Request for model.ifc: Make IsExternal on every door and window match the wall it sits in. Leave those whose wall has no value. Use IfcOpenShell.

First a look at what the model holds.

```python
import ifcopenshell
import ifcopenshell.util.element

model = ifcopenshell.open("model.ifc")
print(model.schema)
seen = {}
for e in model.by_type("IfcDoor") + model.by_type("IfcWindow"):
    if not e.FillsVoids:
        continue
    host = e.FillsVoids[0].RelatingOpeningElement.VoidsElements[0].RelatingBuildingElement
    own = ifcopenshell.util.element.get_pset(e, f"Pset_{e.is_a()[3:].removesuffix('StandardCase')}Common", "IsExternal")
    wall = ifcopenshell.util.element.get_pset(host, "Pset_WallCommon", "IsExternal")
    seen[e.is_a(), own, wall] = seen.get((e.is_a(), own, wall), 0) + 1
for (cls, own, wall), count in sorted(seen.items(), key=str):
    print(count, cls, "IsExternal:", own, "| host wall:", wall)
```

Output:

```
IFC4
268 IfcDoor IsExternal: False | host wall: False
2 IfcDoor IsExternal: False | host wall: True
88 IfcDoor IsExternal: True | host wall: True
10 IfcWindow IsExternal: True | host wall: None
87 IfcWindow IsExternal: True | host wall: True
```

```python
import ifcopenshell
import ifcopenshell.api.pset
import ifcopenshell.util.element

model = ifcopenshell.open("model.ifc")

count = 0
for ifc_class, pset_name in (("IfcDoor", "Pset_DoorCommon"), ("IfcWindow", "Pset_WindowCommon")):
    for e in model.by_type(ifc_class):
        if not e.FillsVoids:
            continue
        host = e.FillsVoids[0].RelatingOpeningElement.VoidsElements[0].RelatingBuildingElement
        external = ifcopenshell.util.element.get_pset(host, "Pset_WallCommon", "IsExternal")
        if external is None or ifcopenshell.util.element.get_pset(e, pset_name, "IsExternal") == external:
            continue
        pset = ifcopenshell.api.pset.add_pset(model, product=e, name=pset_name)
        ifcopenshell.api.pset.edit_pset(model, pset=pset, properties={"IsExternal": external})
        count += 1

print(count, "updated")

model.write("model-out.ifc")
```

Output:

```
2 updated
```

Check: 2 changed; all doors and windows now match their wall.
